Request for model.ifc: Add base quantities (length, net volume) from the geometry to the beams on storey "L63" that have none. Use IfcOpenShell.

First a look at what the model holds.

```python
import ifcopenshell
import ifcopenshell.util.element
import ifcopenshell.util.unit

model = ifcopenshell.open("model.ifc")
print(model.schema)
for unit_type in ("LENGTHUNIT", "AREAUNIT", "VOLUMEUNIT"):
    print(unit_type, ifcopenshell.util.unit.calculate_unit_scale(model, unit_type))
storey = next(s for s in model.by_type("IfcBuildingStorey") if s.Name == "L63")
beams = [e for e in ifcopenshell.util.element.get_decomposition(storey) if e.is_a("IfcBeam")]
for e in sorted(beams, key=lambda e: e.id()):
    print(e.id(), e.is_a(), e.Name, list(ifcopenshell.util.element.get_psets(e, qtos_only=True)), sep=" | ")
```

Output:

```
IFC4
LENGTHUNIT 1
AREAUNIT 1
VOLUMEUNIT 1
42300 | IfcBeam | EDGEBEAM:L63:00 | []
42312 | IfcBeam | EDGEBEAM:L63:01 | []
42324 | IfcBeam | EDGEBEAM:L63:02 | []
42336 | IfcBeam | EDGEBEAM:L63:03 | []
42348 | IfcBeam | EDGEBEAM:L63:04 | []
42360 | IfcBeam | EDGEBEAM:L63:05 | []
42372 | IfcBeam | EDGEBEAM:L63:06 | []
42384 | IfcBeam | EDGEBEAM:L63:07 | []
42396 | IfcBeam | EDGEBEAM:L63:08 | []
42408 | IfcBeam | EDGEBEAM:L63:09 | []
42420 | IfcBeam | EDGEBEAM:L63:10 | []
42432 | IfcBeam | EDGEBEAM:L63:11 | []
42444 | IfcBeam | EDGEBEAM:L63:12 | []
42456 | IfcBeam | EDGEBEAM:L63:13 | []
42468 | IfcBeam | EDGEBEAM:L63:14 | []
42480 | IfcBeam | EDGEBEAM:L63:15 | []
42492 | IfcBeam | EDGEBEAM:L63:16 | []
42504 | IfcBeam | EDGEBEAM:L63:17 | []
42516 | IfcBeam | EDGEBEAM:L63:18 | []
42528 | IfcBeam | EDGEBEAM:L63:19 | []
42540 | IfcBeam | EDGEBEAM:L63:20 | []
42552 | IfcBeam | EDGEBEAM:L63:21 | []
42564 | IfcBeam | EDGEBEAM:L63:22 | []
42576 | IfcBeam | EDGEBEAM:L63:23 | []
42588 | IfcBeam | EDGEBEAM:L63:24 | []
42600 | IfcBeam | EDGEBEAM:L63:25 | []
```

```python
import ifcopenshell
import ifcopenshell.api.pset
import ifcopenshell.geom
import ifcopenshell.util.element
import ifcopenshell.util.shape
import ifcopenshell.util.unit

model = ifcopenshell.open("model.ifc")
unit_scale = ifcopenshell.util.unit.calculate_unit_scale(model)
volume_scale = ifcopenshell.util.unit.calculate_unit_scale(model, "VOLUMEUNIT")
settings = ifcopenshell.geom.settings()

storey = next(s for s in model.by_type("IfcBuildingStorey") if s.Name == "L63")
beams = [e for e in ifcopenshell.util.element.get_decomposition(storey) if e.is_a("IfcBeam")]

for e in sorted(beams, key=lambda e: e.id()):
    if ifcopenshell.util.element.get_psets(e, qtos_only=True, should_inherit=False):
        continue
    # Geometry comes back in metres, in the element's own axes.
    shape = ifcopenshell.geom.create_shape(settings, e)
    values = {
        "Length": ifcopenshell.util.shape.get_max_xyz(shape.geometry) / unit_scale,
        "NetVolume": ifcopenshell.util.shape.get_volume(shape.geometry) / volume_scale,
    }
    qto = ifcopenshell.api.pset.add_qto(model, product=e, name="Qto_BeamBaseQuantities")
    ifcopenshell.api.pset.edit_qto(model, qto=qto, properties=values)
    print(e.id(), {k: round(v, 3) for k, v in values.items()})

model.write("model_updated.ifc")
```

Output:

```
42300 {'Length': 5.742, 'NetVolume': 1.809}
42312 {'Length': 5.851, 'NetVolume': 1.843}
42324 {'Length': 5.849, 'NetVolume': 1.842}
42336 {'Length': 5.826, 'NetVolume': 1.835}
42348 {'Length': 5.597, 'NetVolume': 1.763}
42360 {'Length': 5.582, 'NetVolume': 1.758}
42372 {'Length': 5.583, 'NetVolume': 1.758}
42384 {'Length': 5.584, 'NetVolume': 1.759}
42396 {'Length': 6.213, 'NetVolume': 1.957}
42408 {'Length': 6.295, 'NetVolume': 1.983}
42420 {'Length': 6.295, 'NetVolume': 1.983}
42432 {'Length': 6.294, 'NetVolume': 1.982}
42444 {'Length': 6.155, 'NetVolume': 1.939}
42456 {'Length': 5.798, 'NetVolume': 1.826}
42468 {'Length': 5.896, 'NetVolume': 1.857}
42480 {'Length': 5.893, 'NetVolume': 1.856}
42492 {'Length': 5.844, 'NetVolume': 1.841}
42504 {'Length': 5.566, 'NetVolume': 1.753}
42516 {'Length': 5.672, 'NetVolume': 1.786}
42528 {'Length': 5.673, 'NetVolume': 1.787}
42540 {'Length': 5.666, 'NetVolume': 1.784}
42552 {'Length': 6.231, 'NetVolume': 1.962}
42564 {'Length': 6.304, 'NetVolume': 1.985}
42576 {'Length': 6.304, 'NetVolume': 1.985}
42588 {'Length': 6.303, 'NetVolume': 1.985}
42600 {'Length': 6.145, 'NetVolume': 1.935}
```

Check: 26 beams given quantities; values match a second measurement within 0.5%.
